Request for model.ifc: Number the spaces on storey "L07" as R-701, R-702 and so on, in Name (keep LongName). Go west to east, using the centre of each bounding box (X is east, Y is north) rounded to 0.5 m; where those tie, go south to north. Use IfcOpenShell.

First a look at what the model holds.

```python
import ifcopenshell
import ifcopenshell.util.element
import ifcopenshell.util.placement

model = ifcopenshell.open("model.ifc")
print(model.schema)
storey = next(s for s in model.by_type("IfcBuildingStorey") if s.Name == "L07")
spaces = [e for e in ifcopenshell.util.element.get_decomposition(storey) if e.is_a("IfcSpace")]
for e in sorted(spaces, key=lambda e: e.id()):
    origin = ifcopenshell.util.placement.get_local_placement(e.ObjectPlacement)[:3, 3]
    print(e.id(), e.Name, e.LongName, origin.round(2) + 0.0, sep=" | ")
```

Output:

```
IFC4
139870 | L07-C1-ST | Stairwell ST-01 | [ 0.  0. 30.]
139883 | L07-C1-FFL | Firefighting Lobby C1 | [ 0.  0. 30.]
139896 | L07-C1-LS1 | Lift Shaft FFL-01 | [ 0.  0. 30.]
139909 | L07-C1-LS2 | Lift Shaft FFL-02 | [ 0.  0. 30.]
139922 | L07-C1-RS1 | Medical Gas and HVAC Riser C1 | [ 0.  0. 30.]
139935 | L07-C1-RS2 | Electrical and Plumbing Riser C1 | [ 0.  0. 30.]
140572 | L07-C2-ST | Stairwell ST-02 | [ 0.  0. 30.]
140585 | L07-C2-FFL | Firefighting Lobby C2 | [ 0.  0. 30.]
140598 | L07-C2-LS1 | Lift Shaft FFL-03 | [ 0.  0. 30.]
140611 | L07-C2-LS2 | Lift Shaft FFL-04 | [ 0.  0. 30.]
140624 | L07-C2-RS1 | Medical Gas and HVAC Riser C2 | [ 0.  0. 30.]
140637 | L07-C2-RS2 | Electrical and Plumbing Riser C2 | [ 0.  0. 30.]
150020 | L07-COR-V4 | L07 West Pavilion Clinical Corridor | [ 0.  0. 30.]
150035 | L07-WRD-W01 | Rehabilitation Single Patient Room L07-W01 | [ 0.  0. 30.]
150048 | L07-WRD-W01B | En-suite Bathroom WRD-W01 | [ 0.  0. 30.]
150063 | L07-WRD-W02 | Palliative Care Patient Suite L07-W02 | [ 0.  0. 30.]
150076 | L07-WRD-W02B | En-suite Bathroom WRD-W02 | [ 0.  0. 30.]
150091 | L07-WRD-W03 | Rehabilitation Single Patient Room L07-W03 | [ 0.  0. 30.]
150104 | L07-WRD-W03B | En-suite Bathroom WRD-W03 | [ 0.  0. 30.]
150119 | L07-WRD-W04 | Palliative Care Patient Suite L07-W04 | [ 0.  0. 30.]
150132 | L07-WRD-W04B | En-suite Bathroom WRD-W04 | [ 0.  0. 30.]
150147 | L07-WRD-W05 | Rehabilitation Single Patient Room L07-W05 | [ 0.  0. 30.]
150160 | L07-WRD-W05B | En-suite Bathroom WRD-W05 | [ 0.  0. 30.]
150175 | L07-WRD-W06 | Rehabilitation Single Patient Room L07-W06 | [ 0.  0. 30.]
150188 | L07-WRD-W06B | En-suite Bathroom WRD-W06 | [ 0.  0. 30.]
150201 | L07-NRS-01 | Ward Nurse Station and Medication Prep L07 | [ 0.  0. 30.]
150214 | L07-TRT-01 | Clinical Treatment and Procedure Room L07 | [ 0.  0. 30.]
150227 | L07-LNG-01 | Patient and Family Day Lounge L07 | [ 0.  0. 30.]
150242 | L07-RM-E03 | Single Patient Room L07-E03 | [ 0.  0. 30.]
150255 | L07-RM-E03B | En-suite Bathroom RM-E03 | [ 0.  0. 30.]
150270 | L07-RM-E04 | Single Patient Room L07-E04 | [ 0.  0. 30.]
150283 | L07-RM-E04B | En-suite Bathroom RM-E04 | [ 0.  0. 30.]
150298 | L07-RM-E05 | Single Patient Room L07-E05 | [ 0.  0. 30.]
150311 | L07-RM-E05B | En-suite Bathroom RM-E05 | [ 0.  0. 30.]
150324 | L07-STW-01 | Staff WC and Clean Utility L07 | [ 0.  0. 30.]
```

```python
import ifcopenshell
import ifcopenshell.geom
import ifcopenshell.util.element
import ifcopenshell.util.shape

model = ifcopenshell.open("model.ifc")
settings = ifcopenshell.geom.settings()
settings.set("use-world-coords", True)


def centre(element):
    shape = ifcopenshell.geom.create_shape(settings, element)
    return ifcopenshell.util.shape.get_bbox_centroid(shape.geometry)


storey = next(s for s in model.by_type("IfcBuildingStorey") if s.Name == "L07")
spaces = [e for e in ifcopenshell.util.element.get_decomposition(storey) if e.is_a("IfcSpace")]

# Insertion points can sit at a corner or the storey origin, so sort by the geometry (in metres).
centres = {e: centre(e) for e in spaces}
spaces.sort(key=lambda e: (round(centres[e][0] / 0.5), centres[e][1]))

for i, e in enumerate(spaces, start=1):
    number = f"R-7{i:02d}"
    e.Name = number
    print(e.id(), number)

model.write("model_rev.ifc")
```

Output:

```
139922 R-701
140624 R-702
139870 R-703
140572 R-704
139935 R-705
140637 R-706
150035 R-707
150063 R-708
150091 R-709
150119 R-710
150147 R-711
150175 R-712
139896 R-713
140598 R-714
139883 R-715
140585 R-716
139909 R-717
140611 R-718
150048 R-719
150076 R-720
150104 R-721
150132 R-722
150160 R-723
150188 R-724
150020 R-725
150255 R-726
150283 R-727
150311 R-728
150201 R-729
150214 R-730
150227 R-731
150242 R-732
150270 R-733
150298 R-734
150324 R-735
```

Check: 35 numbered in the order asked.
